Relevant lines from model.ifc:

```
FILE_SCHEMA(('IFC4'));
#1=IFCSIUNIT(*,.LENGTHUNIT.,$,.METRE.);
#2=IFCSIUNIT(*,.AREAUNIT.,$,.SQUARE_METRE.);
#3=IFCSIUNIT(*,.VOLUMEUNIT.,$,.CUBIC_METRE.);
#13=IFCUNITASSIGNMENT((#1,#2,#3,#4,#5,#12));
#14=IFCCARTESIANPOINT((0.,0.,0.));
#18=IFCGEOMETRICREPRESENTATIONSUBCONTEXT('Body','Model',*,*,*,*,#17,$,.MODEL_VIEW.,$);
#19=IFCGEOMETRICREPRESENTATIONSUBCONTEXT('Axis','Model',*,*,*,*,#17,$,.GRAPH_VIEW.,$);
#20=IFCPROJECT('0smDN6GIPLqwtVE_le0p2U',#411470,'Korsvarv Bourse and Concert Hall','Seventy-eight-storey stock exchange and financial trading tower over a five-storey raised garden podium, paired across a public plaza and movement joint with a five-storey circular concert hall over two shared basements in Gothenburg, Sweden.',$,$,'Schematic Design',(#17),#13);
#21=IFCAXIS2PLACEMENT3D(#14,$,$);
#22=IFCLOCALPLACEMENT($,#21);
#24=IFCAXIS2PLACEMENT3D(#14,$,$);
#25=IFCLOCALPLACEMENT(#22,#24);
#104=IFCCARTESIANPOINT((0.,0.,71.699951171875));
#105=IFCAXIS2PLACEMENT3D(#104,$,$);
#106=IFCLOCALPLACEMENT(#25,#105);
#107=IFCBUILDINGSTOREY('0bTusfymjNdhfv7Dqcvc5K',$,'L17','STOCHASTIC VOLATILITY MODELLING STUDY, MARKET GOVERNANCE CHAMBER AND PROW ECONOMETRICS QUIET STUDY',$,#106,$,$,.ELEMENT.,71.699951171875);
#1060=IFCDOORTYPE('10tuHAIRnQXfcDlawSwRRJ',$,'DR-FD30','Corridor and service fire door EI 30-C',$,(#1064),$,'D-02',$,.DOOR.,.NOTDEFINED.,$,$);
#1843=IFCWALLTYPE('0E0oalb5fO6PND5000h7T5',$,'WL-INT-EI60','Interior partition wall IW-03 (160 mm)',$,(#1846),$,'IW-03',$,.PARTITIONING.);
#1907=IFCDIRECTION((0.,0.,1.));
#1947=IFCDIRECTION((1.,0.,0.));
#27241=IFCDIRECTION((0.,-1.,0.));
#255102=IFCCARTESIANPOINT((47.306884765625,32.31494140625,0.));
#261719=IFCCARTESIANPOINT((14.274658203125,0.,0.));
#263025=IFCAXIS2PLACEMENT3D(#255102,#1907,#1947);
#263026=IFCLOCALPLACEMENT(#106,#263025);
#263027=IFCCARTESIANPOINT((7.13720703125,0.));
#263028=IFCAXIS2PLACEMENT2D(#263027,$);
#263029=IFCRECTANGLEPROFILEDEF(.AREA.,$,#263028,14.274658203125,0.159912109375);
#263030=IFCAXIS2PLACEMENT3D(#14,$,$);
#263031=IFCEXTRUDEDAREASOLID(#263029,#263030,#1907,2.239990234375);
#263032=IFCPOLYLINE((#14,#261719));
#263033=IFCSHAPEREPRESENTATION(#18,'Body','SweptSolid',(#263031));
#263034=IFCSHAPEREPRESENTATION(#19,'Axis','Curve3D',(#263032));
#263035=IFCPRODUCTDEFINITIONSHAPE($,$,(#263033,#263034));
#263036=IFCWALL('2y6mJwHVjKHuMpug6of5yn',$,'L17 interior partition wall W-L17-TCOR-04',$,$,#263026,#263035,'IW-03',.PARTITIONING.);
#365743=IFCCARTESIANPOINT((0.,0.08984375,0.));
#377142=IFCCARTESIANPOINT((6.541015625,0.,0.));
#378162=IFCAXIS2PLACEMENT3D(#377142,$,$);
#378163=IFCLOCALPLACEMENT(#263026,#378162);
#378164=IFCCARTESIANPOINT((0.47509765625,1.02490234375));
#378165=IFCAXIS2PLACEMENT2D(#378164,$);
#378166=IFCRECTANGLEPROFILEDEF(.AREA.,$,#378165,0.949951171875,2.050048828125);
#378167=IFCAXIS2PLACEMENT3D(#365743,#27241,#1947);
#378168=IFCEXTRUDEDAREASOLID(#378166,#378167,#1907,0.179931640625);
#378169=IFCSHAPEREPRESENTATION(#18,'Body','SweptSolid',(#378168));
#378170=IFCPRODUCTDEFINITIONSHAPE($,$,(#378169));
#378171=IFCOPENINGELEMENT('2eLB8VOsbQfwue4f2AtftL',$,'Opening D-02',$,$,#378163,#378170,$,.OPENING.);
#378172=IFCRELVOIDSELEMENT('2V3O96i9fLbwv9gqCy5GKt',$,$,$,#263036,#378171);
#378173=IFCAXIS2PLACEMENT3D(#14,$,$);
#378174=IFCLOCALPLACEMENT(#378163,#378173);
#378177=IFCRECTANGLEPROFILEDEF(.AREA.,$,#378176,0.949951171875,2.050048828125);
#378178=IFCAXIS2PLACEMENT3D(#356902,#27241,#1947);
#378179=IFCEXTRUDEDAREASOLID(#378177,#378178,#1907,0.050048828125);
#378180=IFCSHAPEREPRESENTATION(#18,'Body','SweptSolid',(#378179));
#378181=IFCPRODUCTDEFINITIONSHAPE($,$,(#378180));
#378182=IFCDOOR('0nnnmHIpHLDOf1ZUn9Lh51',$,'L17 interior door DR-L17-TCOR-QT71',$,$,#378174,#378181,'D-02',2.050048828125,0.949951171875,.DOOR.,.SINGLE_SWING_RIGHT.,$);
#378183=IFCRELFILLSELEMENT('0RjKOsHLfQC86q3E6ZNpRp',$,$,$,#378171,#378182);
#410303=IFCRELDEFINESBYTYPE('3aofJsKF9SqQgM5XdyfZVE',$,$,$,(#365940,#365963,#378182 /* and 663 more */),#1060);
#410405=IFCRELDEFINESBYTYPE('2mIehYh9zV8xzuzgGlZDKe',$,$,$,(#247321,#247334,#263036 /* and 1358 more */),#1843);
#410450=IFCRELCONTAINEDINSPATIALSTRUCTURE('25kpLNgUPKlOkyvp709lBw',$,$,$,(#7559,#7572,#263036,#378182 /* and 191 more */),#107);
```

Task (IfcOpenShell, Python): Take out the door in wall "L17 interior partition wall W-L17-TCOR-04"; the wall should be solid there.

```python
import ifcopenshell
import ifcopenshell.api.feature
import ifcopenshell.api.root
import ifcopenshell.geom
import ifcopenshell.util.shape

model = ifcopenshell.open("model.ifc")
settings = ifcopenshell.geom.settings()


def volume(element):
    """Net volume in cubic metres, openings subtracted."""
    shape = ifcopenshell.geom.create_shape(settings, element)
    return ifcopenshell.util.shape.get_volume(shape.geometry)


door = model.by_id(378182)
opening = door.FillsVoids[0].RelatingOpeningElement
wall = opening.VoidsElements[0].RelatingBuildingElement
before = volume(wall)

ifcopenshell.api.root.remove_product(model, product=door)
ifcopenshell.api.feature.remove_feature(model, feature=opening)

after = volume(wall)

print(f"wall volume {before:.3f} -> {after:.3f} m3")

model.write("model_updated.ifc")
```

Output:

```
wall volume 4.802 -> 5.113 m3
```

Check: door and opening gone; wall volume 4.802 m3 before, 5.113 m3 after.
